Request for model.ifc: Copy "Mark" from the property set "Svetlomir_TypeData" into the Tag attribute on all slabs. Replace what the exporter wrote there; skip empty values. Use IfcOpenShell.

First a look at what the model holds.

```python
import ifcopenshell
import ifcopenshell.util.element

model = ifcopenshell.open("model.ifc")
print(model.schema)
slabs = model.by_type("IfcSlab")
print(len(slabs), "slabs")
for e in slabs[:8]:
    source = ifcopenshell.util.element.get_pset(e, "Svetlomir_TypeData", "Mark")
    target = e.Tag
    print(e.id(), repr(source), repr(target), sep=" | ")
```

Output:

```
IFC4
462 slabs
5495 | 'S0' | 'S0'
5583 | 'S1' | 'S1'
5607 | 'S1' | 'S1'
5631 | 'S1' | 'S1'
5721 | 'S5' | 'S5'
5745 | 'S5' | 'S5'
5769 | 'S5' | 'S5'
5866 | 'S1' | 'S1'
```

```python
import ifcopenshell
import ifcopenshell.util.element

model = ifcopenshell.open("model.ifc")

count = 0
for e in model.by_type("IfcSlab"):
    value = ifcopenshell.util.element.get_pset(e, "Svetlomir_TypeData", "Mark")
    current = e.Tag
    if not value or not value.strip() or current == value:
        continue
    e.Tag = value
    count += 1

print(count, "slabs updated")

model.write("model_updated.ifc")
```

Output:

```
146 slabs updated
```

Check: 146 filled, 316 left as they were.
